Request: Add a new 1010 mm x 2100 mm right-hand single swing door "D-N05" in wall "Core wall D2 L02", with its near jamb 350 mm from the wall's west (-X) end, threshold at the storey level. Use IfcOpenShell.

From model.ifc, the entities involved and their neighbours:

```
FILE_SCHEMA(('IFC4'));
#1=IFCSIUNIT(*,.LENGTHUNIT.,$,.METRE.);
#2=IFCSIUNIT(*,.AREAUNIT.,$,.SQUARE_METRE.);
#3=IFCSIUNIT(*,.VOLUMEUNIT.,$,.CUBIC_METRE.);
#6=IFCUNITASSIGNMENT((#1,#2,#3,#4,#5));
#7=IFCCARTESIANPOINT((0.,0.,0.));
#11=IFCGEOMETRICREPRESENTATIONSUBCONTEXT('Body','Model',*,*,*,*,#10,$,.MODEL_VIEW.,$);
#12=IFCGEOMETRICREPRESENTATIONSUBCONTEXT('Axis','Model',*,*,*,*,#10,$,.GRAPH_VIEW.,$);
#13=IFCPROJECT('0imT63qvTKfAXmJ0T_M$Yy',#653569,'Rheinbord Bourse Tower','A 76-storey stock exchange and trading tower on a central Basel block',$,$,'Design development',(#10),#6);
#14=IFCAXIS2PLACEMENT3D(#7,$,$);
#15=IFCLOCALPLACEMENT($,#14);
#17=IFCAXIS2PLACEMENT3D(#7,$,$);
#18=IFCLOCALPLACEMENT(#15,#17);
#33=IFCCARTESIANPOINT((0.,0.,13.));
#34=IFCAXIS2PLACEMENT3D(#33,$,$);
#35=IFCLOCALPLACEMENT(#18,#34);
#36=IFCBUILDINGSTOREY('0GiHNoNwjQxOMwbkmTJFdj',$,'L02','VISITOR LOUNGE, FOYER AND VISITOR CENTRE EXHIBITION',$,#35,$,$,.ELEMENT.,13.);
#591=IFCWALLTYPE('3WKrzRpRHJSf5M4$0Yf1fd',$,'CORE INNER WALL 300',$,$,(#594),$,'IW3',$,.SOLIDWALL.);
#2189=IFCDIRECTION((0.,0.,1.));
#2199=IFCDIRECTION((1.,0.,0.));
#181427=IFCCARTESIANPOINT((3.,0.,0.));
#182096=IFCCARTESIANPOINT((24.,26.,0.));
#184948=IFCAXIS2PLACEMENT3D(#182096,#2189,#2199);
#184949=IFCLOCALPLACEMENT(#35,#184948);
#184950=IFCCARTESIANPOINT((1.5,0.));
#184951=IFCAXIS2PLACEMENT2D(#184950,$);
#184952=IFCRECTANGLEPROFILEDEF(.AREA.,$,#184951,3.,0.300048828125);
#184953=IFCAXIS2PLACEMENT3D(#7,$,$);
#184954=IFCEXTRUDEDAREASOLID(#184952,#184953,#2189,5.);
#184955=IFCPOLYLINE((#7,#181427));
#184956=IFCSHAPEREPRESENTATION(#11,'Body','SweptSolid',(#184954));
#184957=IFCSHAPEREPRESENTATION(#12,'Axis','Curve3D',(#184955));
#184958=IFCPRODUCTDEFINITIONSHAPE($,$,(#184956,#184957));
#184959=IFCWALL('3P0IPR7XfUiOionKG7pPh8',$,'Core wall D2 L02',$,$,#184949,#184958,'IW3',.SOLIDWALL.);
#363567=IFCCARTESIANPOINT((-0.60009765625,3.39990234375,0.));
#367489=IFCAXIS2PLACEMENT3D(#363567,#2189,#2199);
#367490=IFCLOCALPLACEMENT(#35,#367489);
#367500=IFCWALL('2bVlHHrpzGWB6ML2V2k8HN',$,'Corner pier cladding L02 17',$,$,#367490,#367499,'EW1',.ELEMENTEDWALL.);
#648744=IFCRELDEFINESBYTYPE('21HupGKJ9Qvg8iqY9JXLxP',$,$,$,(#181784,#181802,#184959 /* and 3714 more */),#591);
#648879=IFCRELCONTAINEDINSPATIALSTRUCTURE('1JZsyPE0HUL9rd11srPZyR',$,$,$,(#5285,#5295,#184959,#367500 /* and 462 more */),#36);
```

```python
import numpy as np
import ifcopenshell
import ifcopenshell.api.feature
import ifcopenshell.api.geometry
import ifcopenshell.api.root
import ifcopenshell.api.spatial
import ifcopenshell.geom
import ifcopenshell.util.element
import ifcopenshell.util.placement
import ifcopenshell.util.representation
import ifcopenshell.util.shape
import ifcopenshell.util.unit

model = ifcopenshell.open("model.ifc")
unit_scale = ifcopenshell.util.unit.calculate_unit_scale(model)
settings = ifcopenshell.geom.settings()


def volume(element):
    """Net volume in cubic metres, openings subtracted."""
    shape = ifcopenshell.geom.create_shape(settings, element)
    return ifcopenshell.util.shape.get_volume(shape.geometry)


wall = model.by_guid("3P0IPR7XfUiOionKG7pPh8")
storey = ifcopenshell.util.element.get_container(wall, ifc_class="IfcBuildingStorey")
context = ifcopenshell.util.representation.get_context(model, "Model", "Body", "MODEL_VIEW")
before = volume(wall)

width, height, from_end, sill = 1.01, 2.1, 0.35, 0.0  # metres

# The wall runs along its own X axis, and the end named is its -X end.
wall_shape = ifcopenshell.geom.create_shape(settings, wall)
x, y, z = ifcopenshell.util.shape.get_vertices(wall_shape.geometry).T
start = x.min() + from_end
face, thickness = float(y.min()), float(y.max() - y.min())
wall_matrix = ifcopenshell.util.placement.get_local_placement(wall.ObjectPlacement)
level = ifcopenshell.util.placement.get_local_placement(storey.ObjectPlacement)[2, 3]


def in_wall(x, y):
    """Placement at x, y metres in the wall's axes, at sill height."""
    matrix = wall_matrix.copy()
    matrix[:, 3] = wall_matrix @ np.array([x / unit_scale, y / unit_scale, 0.0, 1.0])
    matrix[2, 3] = level + sill / unit_scale
    return matrix


# Opening: a box that overshoots both wall faces by 50 mm.
opening = ifcopenshell.api.root.create_entity(model, ifc_class="IfcOpeningElement", predefined_type="OPENING")
box = ifcopenshell.api.geometry.add_wall_representation(
    model, context=context, length=width, height=height, thickness=thickness + 0.1
)
ifcopenshell.api.geometry.assign_representation(model, product=opening, representation=box)
ifcopenshell.api.geometry.edit_object_placement(model, product=opening, matrix=in_wall(start, face - 0.05), is_si=False)
ifcopenshell.api.feature.add_feature(model, feature=opening, element=wall)

door = ifcopenshell.api.root.create_entity(model, ifc_class="IfcDoor", name="D-N05", predefined_type="DOOR")
door.OverallWidth, door.OverallHeight = width / unit_scale, height / unit_scale
door.OperationType = "SINGLE_SWING_RIGHT"
body = ifcopenshell.api.geometry.add_door_representation(
    model,
    context=context,
    overall_width=door.OverallWidth,
    overall_height=door.OverallHeight,
    operation_type="SINGLE_SWING_RIGHT",
    lining_properties={"LiningDepth": thickness / unit_scale, "ThresholdDepth": thickness / unit_scale},
)
ifcopenshell.api.geometry.assign_representation(model, product=door, representation=body)
ifcopenshell.api.spatial.assign_container(model, products=[door], relating_structure=storey)
ifcopenshell.api.feature.add_filling(model, opening=opening, element=door)

# The lining spans the wall, so the door starts at the wall face.
ifcopenshell.api.geometry.edit_object_placement(model, product=door, matrix=in_wall(start, face), is_si=False)

after = volume(wall)

print(f"wall volume {before:.3f} -> {after:.3f} m3")

model.write("model_v2.ifc")
```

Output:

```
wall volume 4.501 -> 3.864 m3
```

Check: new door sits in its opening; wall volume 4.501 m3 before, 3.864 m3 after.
